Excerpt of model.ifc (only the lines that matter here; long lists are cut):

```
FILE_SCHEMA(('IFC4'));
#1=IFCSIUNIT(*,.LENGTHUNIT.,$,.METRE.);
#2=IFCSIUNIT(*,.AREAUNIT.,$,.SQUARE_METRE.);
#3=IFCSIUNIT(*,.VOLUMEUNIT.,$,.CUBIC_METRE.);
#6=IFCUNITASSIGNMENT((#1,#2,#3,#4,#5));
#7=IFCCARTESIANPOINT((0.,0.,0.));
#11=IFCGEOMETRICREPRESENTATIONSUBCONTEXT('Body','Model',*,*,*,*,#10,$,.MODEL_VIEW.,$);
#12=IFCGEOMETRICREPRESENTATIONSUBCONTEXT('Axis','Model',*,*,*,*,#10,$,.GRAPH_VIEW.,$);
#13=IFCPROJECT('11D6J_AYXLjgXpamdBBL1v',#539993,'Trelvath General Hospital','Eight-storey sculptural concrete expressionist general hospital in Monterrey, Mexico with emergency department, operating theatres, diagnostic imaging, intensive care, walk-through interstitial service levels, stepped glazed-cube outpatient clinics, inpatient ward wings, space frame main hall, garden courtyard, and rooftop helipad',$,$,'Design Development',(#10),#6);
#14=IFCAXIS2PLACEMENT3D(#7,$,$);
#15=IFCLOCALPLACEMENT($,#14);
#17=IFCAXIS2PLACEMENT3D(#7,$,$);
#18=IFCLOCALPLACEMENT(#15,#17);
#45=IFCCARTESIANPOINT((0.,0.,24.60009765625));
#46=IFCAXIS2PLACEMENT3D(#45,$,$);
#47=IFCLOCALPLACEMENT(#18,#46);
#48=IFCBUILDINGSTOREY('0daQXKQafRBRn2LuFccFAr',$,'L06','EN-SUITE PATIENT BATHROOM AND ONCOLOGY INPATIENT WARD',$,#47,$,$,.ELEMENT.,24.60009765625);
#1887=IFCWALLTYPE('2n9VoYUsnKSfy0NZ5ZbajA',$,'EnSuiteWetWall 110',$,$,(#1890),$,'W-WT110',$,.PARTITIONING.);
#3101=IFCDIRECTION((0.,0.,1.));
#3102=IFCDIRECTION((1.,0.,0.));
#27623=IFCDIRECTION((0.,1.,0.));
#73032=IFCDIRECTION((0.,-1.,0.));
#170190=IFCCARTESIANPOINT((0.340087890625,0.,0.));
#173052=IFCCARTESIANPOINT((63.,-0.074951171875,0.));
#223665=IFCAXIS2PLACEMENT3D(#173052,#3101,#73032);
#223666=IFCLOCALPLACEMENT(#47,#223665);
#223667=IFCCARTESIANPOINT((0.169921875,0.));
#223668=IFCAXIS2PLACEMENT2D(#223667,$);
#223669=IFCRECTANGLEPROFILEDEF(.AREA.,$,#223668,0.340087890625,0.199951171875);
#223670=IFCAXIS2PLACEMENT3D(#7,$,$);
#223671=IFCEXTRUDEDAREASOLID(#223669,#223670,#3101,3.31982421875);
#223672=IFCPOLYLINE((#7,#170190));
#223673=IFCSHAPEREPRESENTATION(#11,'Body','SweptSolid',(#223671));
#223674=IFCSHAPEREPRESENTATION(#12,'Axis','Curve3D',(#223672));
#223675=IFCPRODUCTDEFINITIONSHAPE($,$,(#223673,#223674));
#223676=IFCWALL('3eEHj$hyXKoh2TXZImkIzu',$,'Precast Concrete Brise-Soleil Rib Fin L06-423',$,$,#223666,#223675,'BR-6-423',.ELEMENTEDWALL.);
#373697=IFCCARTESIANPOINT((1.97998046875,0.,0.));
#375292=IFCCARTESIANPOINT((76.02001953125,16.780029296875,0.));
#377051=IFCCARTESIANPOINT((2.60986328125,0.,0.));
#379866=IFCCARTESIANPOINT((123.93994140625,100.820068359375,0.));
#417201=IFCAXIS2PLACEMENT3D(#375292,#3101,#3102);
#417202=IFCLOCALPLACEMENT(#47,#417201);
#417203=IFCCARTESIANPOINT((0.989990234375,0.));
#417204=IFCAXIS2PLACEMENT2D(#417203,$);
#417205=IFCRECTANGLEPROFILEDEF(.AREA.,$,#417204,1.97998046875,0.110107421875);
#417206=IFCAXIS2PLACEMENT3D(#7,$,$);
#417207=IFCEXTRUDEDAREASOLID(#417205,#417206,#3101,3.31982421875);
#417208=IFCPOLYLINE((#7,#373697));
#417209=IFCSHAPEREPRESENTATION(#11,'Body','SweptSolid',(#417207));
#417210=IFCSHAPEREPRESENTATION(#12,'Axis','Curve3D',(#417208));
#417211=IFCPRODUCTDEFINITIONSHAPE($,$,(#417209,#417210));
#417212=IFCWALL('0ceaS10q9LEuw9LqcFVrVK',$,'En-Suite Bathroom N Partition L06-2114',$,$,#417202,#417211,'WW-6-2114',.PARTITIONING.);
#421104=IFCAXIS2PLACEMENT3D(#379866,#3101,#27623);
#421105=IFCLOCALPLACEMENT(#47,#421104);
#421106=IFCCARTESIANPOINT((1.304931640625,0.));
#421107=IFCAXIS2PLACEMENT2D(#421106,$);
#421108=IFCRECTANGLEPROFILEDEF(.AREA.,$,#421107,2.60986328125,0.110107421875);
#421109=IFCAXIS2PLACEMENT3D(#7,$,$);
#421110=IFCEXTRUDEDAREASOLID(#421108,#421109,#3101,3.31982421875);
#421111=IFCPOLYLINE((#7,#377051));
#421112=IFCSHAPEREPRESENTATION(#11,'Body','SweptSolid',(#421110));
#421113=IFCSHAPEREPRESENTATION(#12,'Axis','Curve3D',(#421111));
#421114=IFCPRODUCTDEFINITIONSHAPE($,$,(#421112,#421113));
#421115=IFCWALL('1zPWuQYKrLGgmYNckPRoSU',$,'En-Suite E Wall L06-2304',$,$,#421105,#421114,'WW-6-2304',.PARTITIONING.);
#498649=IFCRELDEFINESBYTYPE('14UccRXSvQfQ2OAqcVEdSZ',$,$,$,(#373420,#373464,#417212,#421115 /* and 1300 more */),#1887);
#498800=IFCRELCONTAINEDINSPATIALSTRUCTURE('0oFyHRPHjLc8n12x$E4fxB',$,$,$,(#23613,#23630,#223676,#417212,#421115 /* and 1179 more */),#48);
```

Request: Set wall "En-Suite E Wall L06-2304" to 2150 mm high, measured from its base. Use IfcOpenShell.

```python
import ifcopenshell
import ifcopenshell.geom
import ifcopenshell.util.representation
import ifcopenshell.util.shape
import ifcopenshell.util.unit

model = ifcopenshell.open("model.ifc")
unit_scale = ifcopenshell.util.unit.calculate_unit_scale(model)
settings = ifcopenshell.geom.settings()


def volume(element):
    """Net volume in cubic metres, openings subtracted."""
    shape = ifcopenshell.geom.create_shape(settings, element)
    return ifcopenshell.util.shape.get_volume(shape.geometry)


wall = model.by_guid("1zPWuQYKrLGgmYNckPRoSU")
before = volume(wall)

body = ifcopenshell.util.representation.get_representation(wall, "Model", "Body")
solid = body.Items[0]
old_height = solid.Depth
solid.Depth = 2.15 / unit_scale
after = volume(wall)

print(f"height {old_height:g} -> {solid.Depth:g}, volume {before:.3f} -> {after:.3f} m3")

model.write("model-out.ifc")
```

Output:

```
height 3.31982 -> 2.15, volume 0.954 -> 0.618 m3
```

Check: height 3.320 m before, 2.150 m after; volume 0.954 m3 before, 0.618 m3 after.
